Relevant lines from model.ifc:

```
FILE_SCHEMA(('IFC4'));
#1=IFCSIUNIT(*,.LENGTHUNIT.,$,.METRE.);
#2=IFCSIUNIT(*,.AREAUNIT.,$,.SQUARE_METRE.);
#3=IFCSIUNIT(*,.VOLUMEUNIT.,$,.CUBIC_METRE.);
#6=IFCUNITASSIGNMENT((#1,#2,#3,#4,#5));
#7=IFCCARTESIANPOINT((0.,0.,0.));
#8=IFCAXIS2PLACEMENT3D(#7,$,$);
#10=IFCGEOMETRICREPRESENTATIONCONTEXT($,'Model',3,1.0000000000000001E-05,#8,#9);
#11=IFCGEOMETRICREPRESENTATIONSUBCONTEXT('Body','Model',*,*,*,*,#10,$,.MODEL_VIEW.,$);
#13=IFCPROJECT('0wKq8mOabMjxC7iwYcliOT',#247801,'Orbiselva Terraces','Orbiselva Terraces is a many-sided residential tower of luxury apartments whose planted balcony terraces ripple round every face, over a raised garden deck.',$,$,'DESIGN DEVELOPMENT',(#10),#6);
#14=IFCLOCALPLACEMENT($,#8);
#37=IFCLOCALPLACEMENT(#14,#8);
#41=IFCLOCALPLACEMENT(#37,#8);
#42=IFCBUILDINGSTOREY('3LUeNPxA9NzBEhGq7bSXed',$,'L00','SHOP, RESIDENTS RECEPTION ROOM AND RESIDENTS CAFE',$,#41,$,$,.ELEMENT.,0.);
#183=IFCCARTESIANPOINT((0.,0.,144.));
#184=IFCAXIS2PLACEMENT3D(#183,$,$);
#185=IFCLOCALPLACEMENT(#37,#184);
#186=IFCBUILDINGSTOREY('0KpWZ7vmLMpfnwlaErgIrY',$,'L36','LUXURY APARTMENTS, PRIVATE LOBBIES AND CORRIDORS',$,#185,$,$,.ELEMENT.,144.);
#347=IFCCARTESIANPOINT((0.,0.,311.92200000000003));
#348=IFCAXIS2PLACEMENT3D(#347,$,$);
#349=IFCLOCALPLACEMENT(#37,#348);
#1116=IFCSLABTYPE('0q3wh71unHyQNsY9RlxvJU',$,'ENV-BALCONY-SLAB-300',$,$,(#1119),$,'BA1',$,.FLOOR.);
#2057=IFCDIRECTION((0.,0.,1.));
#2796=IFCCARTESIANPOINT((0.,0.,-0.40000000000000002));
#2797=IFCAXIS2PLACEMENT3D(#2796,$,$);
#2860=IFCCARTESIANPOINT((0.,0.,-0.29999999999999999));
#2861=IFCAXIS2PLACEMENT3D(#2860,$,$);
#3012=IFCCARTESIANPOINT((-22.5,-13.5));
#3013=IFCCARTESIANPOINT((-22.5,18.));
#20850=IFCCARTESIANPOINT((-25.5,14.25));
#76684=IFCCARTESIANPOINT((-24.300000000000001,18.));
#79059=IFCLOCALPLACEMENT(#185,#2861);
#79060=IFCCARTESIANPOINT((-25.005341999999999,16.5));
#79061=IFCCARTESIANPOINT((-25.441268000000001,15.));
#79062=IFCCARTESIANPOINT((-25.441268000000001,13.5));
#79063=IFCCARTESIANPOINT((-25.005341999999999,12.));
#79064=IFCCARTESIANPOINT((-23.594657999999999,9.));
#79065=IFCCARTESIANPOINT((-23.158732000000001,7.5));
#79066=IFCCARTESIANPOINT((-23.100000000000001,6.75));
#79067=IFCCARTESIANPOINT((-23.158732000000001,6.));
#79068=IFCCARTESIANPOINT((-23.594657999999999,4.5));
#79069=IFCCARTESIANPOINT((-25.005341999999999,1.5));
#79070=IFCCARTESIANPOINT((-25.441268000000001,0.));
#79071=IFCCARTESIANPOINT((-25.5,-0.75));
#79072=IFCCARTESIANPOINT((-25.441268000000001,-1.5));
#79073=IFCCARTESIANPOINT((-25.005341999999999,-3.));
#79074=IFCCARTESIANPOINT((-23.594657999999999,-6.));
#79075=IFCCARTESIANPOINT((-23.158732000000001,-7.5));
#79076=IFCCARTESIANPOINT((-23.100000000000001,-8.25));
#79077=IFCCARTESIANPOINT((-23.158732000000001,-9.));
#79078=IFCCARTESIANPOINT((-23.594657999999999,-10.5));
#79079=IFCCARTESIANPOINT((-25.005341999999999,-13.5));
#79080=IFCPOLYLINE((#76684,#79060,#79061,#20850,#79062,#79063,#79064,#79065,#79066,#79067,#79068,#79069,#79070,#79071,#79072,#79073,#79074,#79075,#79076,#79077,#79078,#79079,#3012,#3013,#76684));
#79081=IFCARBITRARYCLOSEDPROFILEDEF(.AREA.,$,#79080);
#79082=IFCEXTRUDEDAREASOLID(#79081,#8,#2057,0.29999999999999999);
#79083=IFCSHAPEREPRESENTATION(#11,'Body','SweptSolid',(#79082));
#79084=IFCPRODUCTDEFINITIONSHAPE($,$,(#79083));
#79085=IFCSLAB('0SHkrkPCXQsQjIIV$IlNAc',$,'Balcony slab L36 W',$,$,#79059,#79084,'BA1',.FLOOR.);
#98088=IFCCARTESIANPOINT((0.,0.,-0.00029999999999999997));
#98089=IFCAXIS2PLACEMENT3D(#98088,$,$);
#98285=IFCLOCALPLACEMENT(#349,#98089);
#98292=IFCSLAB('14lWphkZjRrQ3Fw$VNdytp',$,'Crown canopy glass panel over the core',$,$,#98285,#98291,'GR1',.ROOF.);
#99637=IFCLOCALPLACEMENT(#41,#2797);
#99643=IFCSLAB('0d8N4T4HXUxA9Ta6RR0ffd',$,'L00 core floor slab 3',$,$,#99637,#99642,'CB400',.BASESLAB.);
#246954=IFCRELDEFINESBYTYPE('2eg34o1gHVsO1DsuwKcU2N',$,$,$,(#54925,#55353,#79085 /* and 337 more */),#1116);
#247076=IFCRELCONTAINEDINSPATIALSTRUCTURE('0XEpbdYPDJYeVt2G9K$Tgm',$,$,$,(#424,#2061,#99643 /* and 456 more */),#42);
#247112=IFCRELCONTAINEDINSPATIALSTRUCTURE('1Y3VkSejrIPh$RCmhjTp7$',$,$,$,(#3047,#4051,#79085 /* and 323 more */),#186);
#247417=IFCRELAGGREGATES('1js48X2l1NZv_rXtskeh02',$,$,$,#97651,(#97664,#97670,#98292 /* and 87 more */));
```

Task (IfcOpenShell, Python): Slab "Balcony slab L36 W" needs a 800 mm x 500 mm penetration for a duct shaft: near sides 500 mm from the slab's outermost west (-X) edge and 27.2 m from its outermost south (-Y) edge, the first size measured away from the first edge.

```python
import numpy as np
import ifcopenshell
import ifcopenshell.api.feature
import ifcopenshell.api.geometry
import ifcopenshell.api.root
import ifcopenshell.geom
import ifcopenshell.util.placement
import ifcopenshell.util.representation
import ifcopenshell.util.shape
import ifcopenshell.util.unit

model = ifcopenshell.open("model.ifc")
unit_scale = ifcopenshell.util.unit.calculate_unit_scale(model)
settings = ifcopenshell.geom.settings()


def volume(element):
    """Net volume in cubic metres, openings subtracted."""
    shape = ifcopenshell.geom.create_shape(settings, element)
    return ifcopenshell.util.shape.get_volume(shape.geometry)


slab = model.by_id(79085)
before = volume(slab)

# Extent in the slab's own axes, in metres. The edges named are its -X and -Y sides.
slab_shape = ifcopenshell.geom.create_shape(settings, slab)
vertices = ifcopenshell.util.shape.get_vertices(slab_shape.geometry)
x_min, y_min, bottom = vertices.min(axis=0)
top = vertices[:, 2].max()

opening = ifcopenshell.api.root.create_entity(model, ifc_class="IfcOpeningElement", name="Duct shaft opening", predefined_type="OPENING")
context = ifcopenshell.util.representation.get_context(model, "Model", "Body", "MODEL_VIEW")
width, depth = 0.8, 0.5
outline = [(0.0, 0.0), (width, 0.0), (width, depth), (0.0, depth), (0.0, 0.0)]
# Overshoot both faces by 50 mm so the cut is clean.
shape = ifcopenshell.api.geometry.add_slab_representation(
    model, context=context, depth=top - bottom + 0.1, polyline=outline
)
ifcopenshell.api.geometry.assign_representation(model, product=opening, representation=shape)

matrix = ifcopenshell.util.placement.get_local_placement(slab.ObjectPlacement)
matrix[:, 3] = matrix @ np.append(np.array([x_min + 0.5, y_min + 27.2, bottom - 0.05]) / unit_scale, 1.0)
ifcopenshell.api.geometry.edit_object_placement(model, product=opening, matrix=matrix, is_si=False)
ifcopenshell.api.feature.add_feature(model, feature=opening, element=slab)

after = volume(slab)

print(f"slab volume {before:.3f} -> {after:.3f} m3")

model.write("model-out.ifc")
```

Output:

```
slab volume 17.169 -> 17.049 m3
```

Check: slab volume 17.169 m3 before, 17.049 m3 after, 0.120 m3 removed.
